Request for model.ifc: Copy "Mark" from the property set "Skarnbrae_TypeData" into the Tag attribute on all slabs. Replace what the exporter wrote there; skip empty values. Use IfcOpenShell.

First a look at what the model holds.

```python
import ifcopenshell
import ifcopenshell.util.element

model = ifcopenshell.open("model.ifc")
print(model.schema)
slabs = model.by_type("IfcSlab")
print(len(slabs), "slabs")
for e in slabs[:8]:
    source = ifcopenshell.util.element.get_pset(e, "Skarnbrae_TypeData", "Mark")
    target = e.Tag
    print(e.id(), repr(source), repr(target), sep=" | ")
```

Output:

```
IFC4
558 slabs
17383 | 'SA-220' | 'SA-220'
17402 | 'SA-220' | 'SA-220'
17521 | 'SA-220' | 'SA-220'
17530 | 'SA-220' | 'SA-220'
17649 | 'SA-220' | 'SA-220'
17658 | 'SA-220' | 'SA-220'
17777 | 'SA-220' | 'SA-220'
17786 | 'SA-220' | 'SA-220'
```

```python
import ifcopenshell
import ifcopenshell.util.element

model = ifcopenshell.open("model.ifc")

count = 0
for e in model.by_type("IfcSlab"):
    value = ifcopenshell.util.element.get_pset(e, "Skarnbrae_TypeData", "Mark")
    current = e.Tag
    if not value or not value.strip() or current == value:
        continue
    e.Tag = value
    count += 1

print(count, "slabs updated")

model.write("model_updated.ifc")
```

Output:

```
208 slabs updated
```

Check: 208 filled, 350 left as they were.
